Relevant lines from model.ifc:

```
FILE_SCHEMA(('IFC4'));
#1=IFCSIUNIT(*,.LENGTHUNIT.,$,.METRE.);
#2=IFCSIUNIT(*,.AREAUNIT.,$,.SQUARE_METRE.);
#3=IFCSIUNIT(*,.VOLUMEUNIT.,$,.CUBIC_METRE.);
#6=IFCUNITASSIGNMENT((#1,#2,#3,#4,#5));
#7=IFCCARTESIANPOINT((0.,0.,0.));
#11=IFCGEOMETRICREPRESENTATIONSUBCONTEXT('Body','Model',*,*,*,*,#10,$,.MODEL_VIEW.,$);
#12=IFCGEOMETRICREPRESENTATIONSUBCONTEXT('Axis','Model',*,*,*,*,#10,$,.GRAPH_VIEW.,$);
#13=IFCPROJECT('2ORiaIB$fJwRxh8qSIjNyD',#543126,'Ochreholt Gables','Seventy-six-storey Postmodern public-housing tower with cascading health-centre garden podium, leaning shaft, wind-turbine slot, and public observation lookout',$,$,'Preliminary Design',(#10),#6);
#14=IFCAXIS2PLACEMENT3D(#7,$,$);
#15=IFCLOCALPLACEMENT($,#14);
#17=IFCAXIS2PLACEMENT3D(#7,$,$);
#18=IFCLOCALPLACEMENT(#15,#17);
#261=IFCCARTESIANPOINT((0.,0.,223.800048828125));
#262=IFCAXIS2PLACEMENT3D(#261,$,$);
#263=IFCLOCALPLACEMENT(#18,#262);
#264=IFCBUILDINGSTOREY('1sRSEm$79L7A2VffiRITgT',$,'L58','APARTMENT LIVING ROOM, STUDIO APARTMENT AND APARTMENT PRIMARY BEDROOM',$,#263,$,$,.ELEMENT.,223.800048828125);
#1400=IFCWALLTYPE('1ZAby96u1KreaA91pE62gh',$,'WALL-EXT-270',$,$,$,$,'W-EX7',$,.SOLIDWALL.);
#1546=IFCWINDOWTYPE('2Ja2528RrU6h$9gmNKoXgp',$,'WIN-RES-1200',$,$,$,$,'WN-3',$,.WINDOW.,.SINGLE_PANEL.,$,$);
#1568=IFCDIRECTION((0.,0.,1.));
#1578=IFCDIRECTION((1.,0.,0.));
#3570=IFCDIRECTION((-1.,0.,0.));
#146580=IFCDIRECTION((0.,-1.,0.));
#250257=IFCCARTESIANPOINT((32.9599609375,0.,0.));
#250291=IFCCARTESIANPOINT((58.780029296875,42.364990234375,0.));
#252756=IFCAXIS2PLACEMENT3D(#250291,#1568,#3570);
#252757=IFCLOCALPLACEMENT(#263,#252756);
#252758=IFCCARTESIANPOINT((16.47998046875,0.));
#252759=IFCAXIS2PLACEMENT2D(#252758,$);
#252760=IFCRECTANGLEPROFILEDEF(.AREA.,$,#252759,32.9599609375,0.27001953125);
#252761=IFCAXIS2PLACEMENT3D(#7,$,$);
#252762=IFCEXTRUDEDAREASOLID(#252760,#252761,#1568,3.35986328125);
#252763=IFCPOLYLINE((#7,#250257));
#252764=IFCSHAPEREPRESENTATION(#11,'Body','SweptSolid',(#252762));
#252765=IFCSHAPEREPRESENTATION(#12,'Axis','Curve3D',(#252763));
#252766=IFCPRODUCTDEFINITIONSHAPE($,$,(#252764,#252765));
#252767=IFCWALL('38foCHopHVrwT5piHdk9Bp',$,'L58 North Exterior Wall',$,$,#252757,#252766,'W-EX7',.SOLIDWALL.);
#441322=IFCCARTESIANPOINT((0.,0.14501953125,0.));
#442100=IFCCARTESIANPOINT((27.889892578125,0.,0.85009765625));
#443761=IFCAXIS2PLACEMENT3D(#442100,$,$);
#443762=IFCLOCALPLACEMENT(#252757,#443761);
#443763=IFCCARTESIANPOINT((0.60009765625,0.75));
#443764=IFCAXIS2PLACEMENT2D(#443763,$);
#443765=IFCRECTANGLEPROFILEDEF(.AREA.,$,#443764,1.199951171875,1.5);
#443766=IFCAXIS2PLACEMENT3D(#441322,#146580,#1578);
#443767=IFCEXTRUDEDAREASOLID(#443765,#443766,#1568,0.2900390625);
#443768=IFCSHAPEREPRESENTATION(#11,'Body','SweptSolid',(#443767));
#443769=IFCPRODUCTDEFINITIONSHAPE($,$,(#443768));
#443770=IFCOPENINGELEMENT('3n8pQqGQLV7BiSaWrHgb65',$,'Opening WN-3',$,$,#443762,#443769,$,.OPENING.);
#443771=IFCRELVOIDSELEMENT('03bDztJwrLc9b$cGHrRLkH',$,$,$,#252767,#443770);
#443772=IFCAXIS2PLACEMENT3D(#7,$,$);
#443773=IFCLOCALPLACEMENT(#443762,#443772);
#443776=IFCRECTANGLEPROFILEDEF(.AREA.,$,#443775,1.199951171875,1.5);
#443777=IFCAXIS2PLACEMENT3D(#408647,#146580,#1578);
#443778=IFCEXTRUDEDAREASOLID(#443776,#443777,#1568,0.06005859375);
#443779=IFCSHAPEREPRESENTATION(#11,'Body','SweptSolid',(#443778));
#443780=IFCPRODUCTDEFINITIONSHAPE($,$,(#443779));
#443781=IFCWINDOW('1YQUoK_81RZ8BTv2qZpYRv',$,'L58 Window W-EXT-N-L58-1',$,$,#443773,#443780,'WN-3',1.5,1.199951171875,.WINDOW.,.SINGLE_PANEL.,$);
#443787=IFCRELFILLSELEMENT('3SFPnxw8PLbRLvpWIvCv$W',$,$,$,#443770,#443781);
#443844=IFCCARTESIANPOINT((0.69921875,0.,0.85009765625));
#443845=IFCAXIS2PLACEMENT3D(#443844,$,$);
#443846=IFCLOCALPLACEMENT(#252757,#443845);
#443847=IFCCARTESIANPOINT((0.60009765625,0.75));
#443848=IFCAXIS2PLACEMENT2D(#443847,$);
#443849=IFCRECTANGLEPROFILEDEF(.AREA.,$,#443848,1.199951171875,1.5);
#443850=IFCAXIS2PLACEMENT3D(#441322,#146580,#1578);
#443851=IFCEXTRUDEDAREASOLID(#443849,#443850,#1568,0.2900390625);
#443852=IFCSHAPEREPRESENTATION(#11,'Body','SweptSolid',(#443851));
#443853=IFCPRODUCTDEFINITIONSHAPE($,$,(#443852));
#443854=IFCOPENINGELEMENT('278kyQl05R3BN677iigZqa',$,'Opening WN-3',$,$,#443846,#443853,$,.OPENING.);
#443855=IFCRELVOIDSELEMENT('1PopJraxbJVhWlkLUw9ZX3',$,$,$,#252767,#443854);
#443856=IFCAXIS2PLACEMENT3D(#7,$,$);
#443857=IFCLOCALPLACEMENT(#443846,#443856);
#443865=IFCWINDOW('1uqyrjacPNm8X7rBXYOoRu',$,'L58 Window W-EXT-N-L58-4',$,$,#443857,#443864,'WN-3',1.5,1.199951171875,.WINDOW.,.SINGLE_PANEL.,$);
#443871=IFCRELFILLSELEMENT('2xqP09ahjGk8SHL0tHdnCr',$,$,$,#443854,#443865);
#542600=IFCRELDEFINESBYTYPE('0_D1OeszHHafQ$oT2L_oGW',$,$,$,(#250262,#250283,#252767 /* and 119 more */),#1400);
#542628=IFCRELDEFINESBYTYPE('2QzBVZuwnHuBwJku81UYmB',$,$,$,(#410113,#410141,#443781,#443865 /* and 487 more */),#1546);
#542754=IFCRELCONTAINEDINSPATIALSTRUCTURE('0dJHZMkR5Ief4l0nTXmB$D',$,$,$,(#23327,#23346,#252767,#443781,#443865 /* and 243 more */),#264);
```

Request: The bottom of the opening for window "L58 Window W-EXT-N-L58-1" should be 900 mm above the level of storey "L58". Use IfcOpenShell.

```python
import numpy as np
import ifcopenshell
import ifcopenshell.api.geometry
import ifcopenshell.geom
import ifcopenshell.util.element
import ifcopenshell.util.placement
import ifcopenshell.util.shape
import ifcopenshell.util.unit

model = ifcopenshell.open("model.ifc")
unit_scale = ifcopenshell.util.unit.calculate_unit_scale(model)

window = model.by_id(443781)
opening = window.FillsVoids[0].RelatingOpeningElement
storey = ifcopenshell.util.element.get_container(window, ifc_class="IfcBuildingStorey")
level = ifcopenshell.util.placement.get_local_placement(storey.ObjectPlacement)[2, 3]

# The opening's origin need not be at the sill, so measure its lowest point.
shape = ifcopenshell.geom.create_shape(ifcopenshell.geom.settings(), opening)
bottom = ifcopenshell.util.shape.get_shape_bottom_elevation(shape, shape.geometry) / unit_scale
dz = level + 0.9 / unit_scale - bottom

shift = np.array([0.0, 0.0, dz])
# The window is placed relative to its opening, so it follows when the opening moves.
matrix = ifcopenshell.util.placement.get_local_placement(opening.ObjectPlacement)
matrix[:3, 3] += shift
ifcopenshell.api.geometry.edit_object_placement(
    model, product=opening, matrix=matrix, is_si=False, should_transform_children=True
)

print(f"moved by {dz * unit_scale:+.3f} m")

model.write("model_rev.ifc")
```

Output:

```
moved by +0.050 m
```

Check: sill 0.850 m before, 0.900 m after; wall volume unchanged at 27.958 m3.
